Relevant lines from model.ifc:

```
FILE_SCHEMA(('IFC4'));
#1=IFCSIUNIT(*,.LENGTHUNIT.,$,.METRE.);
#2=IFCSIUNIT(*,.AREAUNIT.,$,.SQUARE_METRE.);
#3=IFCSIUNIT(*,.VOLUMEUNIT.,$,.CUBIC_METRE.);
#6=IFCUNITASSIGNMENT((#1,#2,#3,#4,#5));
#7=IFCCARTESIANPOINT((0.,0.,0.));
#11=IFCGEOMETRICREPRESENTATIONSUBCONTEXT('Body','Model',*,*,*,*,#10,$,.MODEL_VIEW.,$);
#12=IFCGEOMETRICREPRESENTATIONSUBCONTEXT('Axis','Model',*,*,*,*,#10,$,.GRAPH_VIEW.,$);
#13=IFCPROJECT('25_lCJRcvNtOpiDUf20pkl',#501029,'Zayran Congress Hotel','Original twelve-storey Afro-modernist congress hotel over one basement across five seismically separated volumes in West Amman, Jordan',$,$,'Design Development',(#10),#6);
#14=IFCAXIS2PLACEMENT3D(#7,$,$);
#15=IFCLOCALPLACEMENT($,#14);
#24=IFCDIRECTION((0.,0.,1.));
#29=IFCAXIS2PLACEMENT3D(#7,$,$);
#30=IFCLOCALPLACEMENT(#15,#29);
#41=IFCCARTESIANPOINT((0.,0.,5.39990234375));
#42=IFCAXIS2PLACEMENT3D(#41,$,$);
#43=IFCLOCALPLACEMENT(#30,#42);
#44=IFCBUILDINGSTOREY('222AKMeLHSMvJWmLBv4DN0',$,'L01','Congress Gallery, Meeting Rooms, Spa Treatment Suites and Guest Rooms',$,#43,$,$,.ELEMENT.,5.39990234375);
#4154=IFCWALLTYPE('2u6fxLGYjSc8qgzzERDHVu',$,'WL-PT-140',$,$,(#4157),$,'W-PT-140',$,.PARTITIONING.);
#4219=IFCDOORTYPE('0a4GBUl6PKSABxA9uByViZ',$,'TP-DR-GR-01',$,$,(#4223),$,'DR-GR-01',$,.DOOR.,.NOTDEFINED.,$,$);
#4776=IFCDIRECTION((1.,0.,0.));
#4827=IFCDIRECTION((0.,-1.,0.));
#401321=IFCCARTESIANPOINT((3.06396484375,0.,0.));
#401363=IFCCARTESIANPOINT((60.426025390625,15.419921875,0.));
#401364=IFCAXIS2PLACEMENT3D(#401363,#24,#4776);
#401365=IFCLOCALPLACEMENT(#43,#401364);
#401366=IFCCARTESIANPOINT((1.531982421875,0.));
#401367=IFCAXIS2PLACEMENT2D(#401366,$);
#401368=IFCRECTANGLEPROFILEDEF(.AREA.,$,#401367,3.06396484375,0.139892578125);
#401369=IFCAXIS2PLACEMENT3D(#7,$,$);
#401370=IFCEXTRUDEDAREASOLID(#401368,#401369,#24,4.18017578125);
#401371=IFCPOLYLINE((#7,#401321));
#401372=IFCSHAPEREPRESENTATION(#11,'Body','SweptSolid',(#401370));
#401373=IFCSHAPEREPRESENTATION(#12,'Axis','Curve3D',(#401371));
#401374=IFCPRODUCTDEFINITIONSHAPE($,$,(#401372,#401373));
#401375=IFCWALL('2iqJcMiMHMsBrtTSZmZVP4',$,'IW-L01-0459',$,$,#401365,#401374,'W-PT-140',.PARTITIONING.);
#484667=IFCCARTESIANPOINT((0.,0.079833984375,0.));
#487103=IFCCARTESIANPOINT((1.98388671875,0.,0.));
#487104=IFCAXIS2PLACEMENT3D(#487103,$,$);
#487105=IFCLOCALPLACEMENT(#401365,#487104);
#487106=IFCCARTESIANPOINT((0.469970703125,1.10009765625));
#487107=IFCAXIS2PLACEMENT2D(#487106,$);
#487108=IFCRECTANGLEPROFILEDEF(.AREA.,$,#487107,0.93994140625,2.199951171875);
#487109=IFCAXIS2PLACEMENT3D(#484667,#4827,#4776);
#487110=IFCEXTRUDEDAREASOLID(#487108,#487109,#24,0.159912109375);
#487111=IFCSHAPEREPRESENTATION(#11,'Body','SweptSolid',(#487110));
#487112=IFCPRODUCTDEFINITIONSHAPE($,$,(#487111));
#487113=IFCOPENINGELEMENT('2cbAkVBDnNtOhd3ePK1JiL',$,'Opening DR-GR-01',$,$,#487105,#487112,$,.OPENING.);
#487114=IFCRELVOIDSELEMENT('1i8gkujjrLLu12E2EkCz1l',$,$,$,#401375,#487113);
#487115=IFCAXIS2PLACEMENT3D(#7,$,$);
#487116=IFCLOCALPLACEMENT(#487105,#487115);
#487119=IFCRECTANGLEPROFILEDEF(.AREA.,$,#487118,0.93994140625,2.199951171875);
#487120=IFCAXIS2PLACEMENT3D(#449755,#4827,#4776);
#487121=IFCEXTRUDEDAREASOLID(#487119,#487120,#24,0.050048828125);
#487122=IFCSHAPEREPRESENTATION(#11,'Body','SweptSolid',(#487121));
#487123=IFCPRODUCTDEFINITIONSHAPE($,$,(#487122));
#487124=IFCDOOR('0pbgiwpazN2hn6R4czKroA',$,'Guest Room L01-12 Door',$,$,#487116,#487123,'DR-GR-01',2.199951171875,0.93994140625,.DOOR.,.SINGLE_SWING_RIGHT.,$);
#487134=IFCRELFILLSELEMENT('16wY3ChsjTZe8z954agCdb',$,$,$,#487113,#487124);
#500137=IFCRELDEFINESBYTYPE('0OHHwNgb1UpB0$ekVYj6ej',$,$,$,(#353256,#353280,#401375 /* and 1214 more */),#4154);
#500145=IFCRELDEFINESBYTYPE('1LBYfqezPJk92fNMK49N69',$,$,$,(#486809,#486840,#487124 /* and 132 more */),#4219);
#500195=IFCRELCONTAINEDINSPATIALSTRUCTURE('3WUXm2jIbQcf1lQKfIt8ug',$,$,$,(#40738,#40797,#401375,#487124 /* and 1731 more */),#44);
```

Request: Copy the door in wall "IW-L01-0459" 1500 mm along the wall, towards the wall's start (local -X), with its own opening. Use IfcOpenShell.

```python
import ifcopenshell
import ifcopenshell.api.feature
import ifcopenshell.api.geometry
import ifcopenshell.api.root
import ifcopenshell.geom
import ifcopenshell.util.element
import ifcopenshell.util.placement
import ifcopenshell.util.shape
import ifcopenshell.util.unit

model = ifcopenshell.open("model.ifc")
unit_scale = ifcopenshell.util.unit.calculate_unit_scale(model)
settings = ifcopenshell.geom.settings()


def volume(element):
    """Net volume in cubic metres, openings subtracted."""
    shape = ifcopenshell.geom.create_shape(settings, element)
    return ifcopenshell.util.shape.get_volume(shape.geometry)


door = model.by_id(487124)
opening = door.FillsVoids[0].RelatingOpeningElement
wall = opening.VoidsElements[0].RelatingBuildingElement
before = volume(wall)
shift = ifcopenshell.util.placement.get_local_placement(wall.ObjectPlacement)[:3, 0] * -1.5 / unit_scale

# copy_class copies the void relationship, type, container and properties, but no geometry.
new_opening = ifcopenshell.api.root.copy_class(model, product=opening)
new_opening.Representation = ifcopenshell.util.element.copy_deep(
    model, opening.Representation, exclude=["IfcGeometricRepresentationContext", "IfcRepresentationMap"]
)
new_door = ifcopenshell.api.root.copy_class(model, product=door)
new_door.Representation = ifcopenshell.util.element.copy_deep(
    model, door.Representation, exclude=["IfcGeometricRepresentationContext", "IfcRepresentationMap"]
)
new_door.Tag = None
ifcopenshell.api.feature.add_filling(model, opening=new_opening, element=new_door)

for old, new in ((opening, new_opening), (door, new_door)):
    matrix = ifcopenshell.util.placement.get_local_placement(old.ObjectPlacement)
    matrix[:3, 3] += shift
    ifcopenshell.api.geometry.edit_object_placement(model, product=new, matrix=matrix, is_si=False)

after = volume(wall)

print(f"wall volume {before:.3f} -> {after:.3f} m3")

model.write("model_updated.ifc")
```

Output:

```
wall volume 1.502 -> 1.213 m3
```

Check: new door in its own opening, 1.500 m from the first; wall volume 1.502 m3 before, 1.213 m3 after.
